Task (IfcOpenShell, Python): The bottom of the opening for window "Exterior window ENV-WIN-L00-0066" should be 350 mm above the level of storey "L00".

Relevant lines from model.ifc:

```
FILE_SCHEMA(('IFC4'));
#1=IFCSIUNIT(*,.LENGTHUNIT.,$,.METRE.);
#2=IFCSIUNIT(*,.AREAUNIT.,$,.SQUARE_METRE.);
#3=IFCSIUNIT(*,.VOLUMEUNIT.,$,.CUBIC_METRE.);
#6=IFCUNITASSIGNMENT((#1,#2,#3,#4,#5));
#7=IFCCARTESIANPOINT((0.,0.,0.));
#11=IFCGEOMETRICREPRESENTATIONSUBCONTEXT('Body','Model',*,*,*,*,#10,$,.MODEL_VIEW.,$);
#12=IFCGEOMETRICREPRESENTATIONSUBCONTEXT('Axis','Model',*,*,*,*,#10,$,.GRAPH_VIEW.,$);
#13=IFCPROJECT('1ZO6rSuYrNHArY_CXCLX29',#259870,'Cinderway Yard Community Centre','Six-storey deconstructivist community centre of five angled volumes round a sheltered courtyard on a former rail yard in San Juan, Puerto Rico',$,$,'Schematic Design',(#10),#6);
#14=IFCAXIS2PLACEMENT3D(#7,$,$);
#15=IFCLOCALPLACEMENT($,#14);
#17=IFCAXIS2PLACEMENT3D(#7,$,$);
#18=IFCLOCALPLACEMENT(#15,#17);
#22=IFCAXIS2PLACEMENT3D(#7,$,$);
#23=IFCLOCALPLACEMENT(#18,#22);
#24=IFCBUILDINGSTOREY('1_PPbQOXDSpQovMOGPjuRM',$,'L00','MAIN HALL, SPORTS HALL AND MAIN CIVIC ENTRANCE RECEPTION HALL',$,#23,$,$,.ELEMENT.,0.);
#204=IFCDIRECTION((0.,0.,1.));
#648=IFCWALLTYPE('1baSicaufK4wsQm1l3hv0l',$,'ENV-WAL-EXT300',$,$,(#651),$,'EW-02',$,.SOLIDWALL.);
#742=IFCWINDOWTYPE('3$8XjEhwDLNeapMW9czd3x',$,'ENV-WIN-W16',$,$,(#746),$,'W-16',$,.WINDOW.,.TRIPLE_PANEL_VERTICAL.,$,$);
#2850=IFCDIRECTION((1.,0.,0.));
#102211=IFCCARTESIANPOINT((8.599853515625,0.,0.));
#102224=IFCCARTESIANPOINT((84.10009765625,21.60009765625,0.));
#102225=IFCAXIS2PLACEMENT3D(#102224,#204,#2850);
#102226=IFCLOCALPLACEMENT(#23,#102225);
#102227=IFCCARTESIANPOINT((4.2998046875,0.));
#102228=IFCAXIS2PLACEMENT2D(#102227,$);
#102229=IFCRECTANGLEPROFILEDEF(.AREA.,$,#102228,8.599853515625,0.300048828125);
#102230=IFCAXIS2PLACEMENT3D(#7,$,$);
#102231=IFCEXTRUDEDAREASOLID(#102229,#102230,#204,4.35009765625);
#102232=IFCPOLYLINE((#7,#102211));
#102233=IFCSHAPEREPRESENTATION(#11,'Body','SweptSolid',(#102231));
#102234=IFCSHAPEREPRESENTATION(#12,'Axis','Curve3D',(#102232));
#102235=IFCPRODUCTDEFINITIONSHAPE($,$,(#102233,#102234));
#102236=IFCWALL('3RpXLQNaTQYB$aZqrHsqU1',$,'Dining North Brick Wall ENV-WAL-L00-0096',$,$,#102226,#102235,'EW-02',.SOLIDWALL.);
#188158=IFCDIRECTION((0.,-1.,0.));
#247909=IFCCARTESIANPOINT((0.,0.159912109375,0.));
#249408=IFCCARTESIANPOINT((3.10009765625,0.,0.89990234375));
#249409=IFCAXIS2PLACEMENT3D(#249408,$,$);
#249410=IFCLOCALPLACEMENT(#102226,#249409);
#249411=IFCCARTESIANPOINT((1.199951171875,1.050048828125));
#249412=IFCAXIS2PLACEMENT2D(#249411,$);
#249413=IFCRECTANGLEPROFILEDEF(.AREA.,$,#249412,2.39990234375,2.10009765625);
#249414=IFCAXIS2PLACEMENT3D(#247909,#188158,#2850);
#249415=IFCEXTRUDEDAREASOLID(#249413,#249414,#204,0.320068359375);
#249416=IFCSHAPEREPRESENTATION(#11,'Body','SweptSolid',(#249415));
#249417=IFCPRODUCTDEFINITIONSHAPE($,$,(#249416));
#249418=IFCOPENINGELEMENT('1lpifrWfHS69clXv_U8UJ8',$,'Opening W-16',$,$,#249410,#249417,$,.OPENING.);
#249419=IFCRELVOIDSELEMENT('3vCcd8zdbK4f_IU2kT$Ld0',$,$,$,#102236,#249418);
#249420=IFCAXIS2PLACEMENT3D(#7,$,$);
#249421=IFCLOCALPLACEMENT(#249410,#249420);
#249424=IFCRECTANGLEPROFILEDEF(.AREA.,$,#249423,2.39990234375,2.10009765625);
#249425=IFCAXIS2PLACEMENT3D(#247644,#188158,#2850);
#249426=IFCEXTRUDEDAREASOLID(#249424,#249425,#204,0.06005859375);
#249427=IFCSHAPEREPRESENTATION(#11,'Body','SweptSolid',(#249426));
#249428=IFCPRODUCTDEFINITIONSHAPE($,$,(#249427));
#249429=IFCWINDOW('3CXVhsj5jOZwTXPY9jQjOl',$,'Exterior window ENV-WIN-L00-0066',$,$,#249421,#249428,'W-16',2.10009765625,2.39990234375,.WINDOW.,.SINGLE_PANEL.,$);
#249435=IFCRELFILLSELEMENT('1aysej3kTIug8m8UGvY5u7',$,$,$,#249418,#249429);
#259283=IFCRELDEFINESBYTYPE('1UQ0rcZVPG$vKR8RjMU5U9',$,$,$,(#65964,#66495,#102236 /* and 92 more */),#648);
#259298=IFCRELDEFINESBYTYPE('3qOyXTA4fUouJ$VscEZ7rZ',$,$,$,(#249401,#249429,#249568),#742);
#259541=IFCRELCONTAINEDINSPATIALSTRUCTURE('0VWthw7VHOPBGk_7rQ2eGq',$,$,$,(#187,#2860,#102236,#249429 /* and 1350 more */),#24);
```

```python
import numpy as np
import ifcopenshell
import ifcopenshell.api.geometry
import ifcopenshell.geom
import ifcopenshell.util.element
import ifcopenshell.util.placement
import ifcopenshell.util.shape
import ifcopenshell.util.unit

model = ifcopenshell.open("model.ifc")
unit_scale = ifcopenshell.util.unit.calculate_unit_scale(model)

window = model.by_id(249429)
opening = window.FillsVoids[0].RelatingOpeningElement
storey = ifcopenshell.util.element.get_container(window, ifc_class="IfcBuildingStorey")
level = ifcopenshell.util.placement.get_local_placement(storey.ObjectPlacement)[2, 3]

# The opening's origin need not be at the sill, so measure its lowest point.
shape = ifcopenshell.geom.create_shape(ifcopenshell.geom.settings(), opening)
bottom = ifcopenshell.util.shape.get_shape_bottom_elevation(shape, shape.geometry) / unit_scale
dz = level + 0.35 - bottom

shift = np.array([0.0, 0.0, dz])
# The window is placed relative to its opening, so it follows when the opening moves.
matrix = ifcopenshell.util.placement.get_local_placement(opening.ObjectPlacement)
matrix[:3, 3] += shift
ifcopenshell.api.geometry.edit_object_placement(
    model, product=opening, matrix=matrix, is_si=False, should_transform_children=True
)

print(f"moved by {dz * unit_scale:+.3f} m")

model.write("model_edited.ifc")
```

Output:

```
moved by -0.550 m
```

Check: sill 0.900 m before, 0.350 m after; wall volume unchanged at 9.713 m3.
